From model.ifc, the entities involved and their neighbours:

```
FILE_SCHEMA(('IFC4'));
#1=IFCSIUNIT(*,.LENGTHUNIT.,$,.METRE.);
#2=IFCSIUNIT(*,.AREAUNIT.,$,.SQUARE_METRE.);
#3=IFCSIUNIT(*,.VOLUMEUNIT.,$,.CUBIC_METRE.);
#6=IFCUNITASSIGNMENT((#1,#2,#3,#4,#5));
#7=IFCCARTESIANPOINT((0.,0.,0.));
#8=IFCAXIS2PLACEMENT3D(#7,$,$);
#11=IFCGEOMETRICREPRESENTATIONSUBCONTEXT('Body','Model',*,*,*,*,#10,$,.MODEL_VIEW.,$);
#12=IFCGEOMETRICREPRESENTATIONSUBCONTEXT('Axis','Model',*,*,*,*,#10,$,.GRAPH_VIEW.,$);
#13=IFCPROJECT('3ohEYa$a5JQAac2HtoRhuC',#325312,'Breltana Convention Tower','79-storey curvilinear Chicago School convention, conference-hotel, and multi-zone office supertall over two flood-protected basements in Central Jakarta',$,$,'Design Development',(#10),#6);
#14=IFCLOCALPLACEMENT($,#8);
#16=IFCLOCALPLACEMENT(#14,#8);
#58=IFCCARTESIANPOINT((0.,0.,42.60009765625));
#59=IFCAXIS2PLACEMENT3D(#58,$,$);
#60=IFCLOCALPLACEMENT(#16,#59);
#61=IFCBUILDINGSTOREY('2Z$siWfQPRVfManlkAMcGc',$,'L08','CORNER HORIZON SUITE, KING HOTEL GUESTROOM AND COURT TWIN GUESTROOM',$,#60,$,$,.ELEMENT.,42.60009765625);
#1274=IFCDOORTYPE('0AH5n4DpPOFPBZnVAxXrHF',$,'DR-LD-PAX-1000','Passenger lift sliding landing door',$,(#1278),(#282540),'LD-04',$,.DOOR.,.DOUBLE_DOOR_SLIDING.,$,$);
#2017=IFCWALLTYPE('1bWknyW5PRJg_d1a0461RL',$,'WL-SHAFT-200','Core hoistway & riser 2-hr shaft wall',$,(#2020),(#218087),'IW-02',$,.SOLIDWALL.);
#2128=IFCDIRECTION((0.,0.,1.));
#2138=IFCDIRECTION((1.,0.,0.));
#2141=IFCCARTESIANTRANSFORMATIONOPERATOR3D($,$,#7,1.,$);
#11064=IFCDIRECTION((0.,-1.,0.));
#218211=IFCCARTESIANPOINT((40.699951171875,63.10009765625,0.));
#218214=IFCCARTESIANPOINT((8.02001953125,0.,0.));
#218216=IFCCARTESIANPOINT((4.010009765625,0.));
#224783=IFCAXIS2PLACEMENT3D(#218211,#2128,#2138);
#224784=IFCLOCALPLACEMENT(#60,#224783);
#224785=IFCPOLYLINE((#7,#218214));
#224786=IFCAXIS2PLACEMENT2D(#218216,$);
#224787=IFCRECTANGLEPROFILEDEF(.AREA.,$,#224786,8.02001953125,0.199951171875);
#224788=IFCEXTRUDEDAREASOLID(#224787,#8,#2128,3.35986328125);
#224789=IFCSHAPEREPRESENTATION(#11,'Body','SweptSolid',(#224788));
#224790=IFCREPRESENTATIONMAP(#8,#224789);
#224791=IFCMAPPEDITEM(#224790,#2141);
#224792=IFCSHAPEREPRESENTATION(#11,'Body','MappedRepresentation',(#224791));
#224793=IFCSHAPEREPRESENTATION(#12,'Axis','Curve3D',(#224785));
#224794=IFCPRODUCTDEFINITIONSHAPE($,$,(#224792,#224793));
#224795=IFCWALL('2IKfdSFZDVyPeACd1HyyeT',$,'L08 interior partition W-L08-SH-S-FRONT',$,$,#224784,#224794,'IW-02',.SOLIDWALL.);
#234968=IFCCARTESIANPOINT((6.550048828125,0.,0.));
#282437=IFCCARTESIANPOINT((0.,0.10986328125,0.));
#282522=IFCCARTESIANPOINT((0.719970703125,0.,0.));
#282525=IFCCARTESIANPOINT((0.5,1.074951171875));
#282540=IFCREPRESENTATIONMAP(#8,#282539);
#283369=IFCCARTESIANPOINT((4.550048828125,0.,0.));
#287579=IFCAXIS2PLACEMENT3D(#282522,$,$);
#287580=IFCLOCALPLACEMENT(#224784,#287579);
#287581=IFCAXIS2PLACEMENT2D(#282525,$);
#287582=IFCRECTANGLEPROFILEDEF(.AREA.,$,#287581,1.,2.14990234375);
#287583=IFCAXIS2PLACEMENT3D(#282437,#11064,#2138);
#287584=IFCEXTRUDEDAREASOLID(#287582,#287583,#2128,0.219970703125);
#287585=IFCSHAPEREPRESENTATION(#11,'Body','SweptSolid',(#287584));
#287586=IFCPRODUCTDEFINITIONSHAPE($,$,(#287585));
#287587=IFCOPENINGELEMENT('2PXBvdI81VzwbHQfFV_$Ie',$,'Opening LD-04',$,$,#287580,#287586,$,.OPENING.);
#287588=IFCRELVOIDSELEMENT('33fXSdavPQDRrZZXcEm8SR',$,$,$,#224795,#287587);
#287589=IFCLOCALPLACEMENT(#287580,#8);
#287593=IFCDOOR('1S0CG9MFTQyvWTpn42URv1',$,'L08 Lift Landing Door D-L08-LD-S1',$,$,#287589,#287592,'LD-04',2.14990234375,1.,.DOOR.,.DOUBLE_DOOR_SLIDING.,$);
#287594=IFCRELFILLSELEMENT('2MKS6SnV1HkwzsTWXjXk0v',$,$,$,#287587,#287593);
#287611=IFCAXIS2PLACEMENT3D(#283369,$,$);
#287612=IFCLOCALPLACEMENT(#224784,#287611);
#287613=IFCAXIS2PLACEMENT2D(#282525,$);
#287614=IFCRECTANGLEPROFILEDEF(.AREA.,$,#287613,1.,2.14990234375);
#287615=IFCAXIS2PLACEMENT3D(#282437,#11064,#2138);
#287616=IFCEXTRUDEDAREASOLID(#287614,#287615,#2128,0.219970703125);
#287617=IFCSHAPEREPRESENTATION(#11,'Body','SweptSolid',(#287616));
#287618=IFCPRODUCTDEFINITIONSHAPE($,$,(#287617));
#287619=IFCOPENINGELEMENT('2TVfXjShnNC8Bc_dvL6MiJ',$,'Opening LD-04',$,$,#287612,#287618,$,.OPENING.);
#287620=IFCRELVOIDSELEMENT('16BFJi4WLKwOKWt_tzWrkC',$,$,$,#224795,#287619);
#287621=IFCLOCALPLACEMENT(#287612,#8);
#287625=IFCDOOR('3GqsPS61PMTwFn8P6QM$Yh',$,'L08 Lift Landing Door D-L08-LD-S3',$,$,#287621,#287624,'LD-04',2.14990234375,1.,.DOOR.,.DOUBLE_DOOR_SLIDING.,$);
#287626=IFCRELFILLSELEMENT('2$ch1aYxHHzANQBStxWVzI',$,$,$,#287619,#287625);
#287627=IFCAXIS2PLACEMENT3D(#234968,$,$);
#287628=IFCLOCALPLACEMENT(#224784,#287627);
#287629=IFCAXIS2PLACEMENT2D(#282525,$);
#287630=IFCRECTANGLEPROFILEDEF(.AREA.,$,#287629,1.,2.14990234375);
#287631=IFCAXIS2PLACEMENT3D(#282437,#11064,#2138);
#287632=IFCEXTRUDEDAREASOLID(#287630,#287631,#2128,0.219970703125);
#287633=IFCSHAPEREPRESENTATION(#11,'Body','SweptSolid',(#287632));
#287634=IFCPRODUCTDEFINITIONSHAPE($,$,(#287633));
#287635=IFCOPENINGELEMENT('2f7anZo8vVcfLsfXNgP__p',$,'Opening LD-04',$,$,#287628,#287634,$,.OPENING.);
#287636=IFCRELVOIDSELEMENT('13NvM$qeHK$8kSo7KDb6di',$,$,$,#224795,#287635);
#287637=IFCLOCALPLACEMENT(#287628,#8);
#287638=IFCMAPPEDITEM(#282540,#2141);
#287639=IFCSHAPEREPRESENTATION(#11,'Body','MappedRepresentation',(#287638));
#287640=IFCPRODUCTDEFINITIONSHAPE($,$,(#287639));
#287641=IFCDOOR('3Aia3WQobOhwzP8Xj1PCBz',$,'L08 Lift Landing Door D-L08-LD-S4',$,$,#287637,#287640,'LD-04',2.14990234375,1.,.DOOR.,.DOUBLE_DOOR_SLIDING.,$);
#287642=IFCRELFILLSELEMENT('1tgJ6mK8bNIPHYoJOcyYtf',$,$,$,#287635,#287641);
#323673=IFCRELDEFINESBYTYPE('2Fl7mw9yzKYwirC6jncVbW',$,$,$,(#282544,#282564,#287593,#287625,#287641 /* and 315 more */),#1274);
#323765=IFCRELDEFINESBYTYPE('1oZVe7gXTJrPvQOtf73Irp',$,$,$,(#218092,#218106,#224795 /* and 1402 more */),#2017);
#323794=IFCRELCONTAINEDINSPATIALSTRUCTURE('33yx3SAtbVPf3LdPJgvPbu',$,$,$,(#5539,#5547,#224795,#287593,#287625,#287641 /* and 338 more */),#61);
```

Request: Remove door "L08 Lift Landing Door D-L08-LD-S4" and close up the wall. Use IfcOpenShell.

```python
import ifcopenshell
import ifcopenshell.api.feature
import ifcopenshell.api.root
import ifcopenshell.geom
import ifcopenshell.util.shape

model = ifcopenshell.open("model.ifc")
settings = ifcopenshell.geom.settings()


def volume(element):
    """Net volume in cubic metres, openings subtracted."""
    shape = ifcopenshell.geom.create_shape(settings, element)
    return ifcopenshell.util.shape.get_volume(shape.geometry)


door = model.by_id(287641)
opening = door.FillsVoids[0].RelatingOpeningElement
wall = opening.VoidsElements[0].RelatingBuildingElement
before = volume(wall)

ifcopenshell.api.root.remove_product(model, product=door)
ifcopenshell.api.feature.remove_feature(model, feature=opening)

after = volume(wall)

print(f"wall volume {before:.3f} -> {after:.3f} m3")

model.write("model-out.ifc")
```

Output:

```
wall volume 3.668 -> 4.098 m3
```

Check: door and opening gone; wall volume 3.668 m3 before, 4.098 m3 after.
